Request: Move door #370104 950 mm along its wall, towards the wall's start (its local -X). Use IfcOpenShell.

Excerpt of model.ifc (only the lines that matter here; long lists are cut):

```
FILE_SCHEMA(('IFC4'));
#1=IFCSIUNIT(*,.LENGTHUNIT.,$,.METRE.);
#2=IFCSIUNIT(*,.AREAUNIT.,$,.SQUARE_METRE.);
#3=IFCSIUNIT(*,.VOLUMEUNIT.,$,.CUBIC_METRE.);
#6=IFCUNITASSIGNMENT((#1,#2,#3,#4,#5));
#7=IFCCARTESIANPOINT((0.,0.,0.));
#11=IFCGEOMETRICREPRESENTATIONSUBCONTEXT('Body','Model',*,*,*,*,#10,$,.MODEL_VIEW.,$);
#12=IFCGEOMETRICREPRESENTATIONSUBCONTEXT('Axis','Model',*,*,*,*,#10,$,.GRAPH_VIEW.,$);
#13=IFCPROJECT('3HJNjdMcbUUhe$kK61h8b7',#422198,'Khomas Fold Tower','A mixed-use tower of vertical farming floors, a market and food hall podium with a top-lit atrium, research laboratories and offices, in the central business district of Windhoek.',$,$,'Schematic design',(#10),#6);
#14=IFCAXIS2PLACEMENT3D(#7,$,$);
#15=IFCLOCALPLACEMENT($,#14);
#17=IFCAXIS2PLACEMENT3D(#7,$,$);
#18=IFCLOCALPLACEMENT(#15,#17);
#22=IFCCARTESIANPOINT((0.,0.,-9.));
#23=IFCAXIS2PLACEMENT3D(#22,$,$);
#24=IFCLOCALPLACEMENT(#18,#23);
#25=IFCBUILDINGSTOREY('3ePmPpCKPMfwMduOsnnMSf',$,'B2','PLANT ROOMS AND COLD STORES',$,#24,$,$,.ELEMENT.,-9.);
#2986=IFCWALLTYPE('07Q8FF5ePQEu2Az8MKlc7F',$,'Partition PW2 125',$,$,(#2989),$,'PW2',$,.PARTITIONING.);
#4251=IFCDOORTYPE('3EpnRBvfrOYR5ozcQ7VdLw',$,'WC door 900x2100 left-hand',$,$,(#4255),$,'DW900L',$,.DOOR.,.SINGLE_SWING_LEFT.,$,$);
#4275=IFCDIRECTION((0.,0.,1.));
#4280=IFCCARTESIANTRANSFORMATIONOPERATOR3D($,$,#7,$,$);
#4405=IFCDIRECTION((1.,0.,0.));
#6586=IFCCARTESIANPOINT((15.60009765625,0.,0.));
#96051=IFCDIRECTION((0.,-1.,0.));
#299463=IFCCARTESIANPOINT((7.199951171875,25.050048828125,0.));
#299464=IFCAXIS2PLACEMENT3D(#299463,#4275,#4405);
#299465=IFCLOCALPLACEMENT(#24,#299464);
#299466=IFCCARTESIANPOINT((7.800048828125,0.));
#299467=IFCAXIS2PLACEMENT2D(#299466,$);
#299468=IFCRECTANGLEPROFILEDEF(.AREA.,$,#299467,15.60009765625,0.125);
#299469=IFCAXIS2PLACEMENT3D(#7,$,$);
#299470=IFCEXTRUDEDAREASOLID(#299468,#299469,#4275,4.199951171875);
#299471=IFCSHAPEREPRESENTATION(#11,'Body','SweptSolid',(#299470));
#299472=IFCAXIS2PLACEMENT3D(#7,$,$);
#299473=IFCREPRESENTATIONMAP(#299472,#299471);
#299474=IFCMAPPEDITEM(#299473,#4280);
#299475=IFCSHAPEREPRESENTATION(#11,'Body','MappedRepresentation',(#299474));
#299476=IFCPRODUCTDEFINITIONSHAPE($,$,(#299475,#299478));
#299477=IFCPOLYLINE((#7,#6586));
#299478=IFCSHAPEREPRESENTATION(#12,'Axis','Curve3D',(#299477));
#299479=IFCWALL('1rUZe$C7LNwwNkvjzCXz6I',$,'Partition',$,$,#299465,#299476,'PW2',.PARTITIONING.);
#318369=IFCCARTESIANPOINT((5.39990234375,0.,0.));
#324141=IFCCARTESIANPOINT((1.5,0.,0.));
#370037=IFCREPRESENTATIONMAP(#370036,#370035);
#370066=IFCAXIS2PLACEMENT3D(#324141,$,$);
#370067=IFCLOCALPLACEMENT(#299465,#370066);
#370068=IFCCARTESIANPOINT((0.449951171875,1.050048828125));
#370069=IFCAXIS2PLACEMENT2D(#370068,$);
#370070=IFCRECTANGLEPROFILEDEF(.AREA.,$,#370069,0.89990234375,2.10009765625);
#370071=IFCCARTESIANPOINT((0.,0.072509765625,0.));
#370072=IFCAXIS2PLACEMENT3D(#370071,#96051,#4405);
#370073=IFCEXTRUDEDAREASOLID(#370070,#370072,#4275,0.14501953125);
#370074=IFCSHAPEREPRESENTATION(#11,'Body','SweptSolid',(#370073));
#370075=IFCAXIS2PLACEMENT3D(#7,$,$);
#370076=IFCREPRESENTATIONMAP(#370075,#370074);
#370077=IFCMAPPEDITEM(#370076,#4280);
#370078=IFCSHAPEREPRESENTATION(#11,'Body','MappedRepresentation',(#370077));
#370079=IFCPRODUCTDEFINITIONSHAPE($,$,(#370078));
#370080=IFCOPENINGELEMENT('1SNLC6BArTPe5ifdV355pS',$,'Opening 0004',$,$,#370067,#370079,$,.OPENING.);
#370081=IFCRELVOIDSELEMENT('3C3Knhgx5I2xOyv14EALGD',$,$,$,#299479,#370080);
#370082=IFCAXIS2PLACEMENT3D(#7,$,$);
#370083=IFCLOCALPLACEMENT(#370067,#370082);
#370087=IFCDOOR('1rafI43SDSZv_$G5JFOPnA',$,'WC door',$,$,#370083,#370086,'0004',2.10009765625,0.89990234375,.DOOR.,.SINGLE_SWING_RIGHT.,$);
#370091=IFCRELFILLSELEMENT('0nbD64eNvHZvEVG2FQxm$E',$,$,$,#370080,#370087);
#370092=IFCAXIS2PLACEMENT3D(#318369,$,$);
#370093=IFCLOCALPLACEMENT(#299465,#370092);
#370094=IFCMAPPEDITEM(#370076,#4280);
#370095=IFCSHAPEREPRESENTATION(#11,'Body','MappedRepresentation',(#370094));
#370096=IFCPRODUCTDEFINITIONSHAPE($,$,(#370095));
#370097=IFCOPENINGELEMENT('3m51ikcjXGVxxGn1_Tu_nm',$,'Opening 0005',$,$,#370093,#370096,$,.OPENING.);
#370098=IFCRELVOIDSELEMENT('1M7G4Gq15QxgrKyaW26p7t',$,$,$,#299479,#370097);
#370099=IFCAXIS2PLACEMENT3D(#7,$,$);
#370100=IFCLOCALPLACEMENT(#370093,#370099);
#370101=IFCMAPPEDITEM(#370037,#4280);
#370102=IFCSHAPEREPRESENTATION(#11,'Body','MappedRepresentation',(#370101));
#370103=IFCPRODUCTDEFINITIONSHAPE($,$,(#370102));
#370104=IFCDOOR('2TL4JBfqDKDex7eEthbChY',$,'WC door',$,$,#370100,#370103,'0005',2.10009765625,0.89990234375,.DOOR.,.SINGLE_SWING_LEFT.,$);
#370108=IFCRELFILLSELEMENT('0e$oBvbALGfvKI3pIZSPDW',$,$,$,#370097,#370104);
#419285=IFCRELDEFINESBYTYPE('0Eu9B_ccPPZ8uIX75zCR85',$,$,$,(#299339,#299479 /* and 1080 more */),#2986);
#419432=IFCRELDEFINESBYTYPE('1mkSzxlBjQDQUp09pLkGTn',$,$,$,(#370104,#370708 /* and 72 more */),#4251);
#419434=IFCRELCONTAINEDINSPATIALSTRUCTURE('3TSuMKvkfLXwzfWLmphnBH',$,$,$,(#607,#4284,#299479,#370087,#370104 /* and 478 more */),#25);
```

```python
import ifcopenshell
import ifcopenshell.api.geometry
import ifcopenshell.util.placement

model = ifcopenshell.open("model.ifc")

door = model.by_guid("2TL4JBfqDKDex7eEthbChY")
opening = door.FillsVoids[0].RelatingOpeningElement
wall = opening.VoidsElements[0].RelatingBuildingElement

wall_matrix = ifcopenshell.util.placement.get_local_placement(wall.ObjectPlacement)
shift = wall_matrix[:3, 0] * -0.95
before = ifcopenshell.util.placement.get_local_placement(door.ObjectPlacement)[:3, 3].copy()

# The door is placed relative to its opening, so it follows when the opening moves.
matrix = ifcopenshell.util.placement.get_local_placement(opening.ObjectPlacement)
matrix[:3, 3] += shift
ifcopenshell.api.geometry.edit_object_placement(
    model, product=opening, matrix=matrix, is_si=False, should_transform_children=True
)

after = ifcopenshell.util.placement.get_local_placement(door.ObjectPlacement)[:3, 3]
print("door moved by", (after - before).round(3) + 0.0)

model.write("model_updated.ifc")
```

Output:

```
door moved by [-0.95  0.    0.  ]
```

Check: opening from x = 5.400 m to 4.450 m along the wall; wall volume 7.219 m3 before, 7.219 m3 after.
